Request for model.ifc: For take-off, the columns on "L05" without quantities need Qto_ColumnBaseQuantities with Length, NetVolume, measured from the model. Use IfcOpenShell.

First a look at what the model holds.

```python
import ifcopenshell
import ifcopenshell.util.element
import ifcopenshell.util.unit

model = ifcopenshell.open("model.ifc")
print(model.schema)
for unit_type in ("LENGTHUNIT", "AREAUNIT", "VOLUMEUNIT"):
    print(unit_type, ifcopenshell.util.unit.calculate_unit_scale(model, unit_type))
storey = next(s for s in model.by_type("IfcBuildingStorey") if s.Name == "L05")
columns = [e for e in ifcopenshell.util.element.get_decomposition(storey) if e.is_a("IfcColumn")]
for e in sorted(columns, key=lambda e: e.id()):
    print(e.id(), e.is_a(), e.Name, list(ifcopenshell.util.element.get_psets(e, qtos_only=True)), sep=" | ")
```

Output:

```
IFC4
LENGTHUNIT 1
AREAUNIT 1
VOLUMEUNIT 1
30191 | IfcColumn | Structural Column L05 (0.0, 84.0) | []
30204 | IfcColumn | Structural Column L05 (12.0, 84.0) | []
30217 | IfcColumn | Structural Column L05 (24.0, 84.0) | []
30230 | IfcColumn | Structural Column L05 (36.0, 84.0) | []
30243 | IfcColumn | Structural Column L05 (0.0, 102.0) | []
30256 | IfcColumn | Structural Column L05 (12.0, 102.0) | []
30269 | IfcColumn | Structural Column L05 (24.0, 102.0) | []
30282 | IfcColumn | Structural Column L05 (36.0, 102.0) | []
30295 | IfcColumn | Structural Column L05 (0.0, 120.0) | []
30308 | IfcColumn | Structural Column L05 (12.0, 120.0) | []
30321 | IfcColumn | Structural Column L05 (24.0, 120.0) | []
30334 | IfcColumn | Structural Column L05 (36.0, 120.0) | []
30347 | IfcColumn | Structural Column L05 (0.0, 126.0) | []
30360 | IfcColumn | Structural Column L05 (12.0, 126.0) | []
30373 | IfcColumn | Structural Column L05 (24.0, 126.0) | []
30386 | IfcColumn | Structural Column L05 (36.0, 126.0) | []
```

```python
import ifcopenshell
import ifcopenshell.api.pset
import ifcopenshell.geom
import ifcopenshell.util.element
import ifcopenshell.util.shape
import ifcopenshell.util.unit

model = ifcopenshell.open("model.ifc")
unit_scale = ifcopenshell.util.unit.calculate_unit_scale(model)
volume_scale = ifcopenshell.util.unit.calculate_unit_scale(model, "VOLUMEUNIT")
settings = ifcopenshell.geom.settings()

storey = next(s for s in model.by_type("IfcBuildingStorey") if s.Name == "L05")
columns = [e for e in ifcopenshell.util.element.get_decomposition(storey) if e.is_a("IfcColumn")]

for e in sorted(columns, key=lambda e: e.id()):
    if ifcopenshell.util.element.get_psets(e, qtos_only=True, should_inherit=False):
        continue
    # Geometry comes back in metres, in the element's own axes.
    shape = ifcopenshell.geom.create_shape(settings, e)
    values = {
        "Length": ifcopenshell.util.shape.get_z(shape.geometry) / unit_scale,
        "NetVolume": ifcopenshell.util.shape.get_volume(shape.geometry) / volume_scale,
    }
    qto = ifcopenshell.api.pset.add_qto(model, product=e, name="Qto_ColumnBaseQuantities")
    ifcopenshell.api.pset.edit_qto(model, qto=qto, properties=values)
    print(e.id(), {k: round(v, 3) for k, v in values.items()})

model.write("model_edited.ifc")
```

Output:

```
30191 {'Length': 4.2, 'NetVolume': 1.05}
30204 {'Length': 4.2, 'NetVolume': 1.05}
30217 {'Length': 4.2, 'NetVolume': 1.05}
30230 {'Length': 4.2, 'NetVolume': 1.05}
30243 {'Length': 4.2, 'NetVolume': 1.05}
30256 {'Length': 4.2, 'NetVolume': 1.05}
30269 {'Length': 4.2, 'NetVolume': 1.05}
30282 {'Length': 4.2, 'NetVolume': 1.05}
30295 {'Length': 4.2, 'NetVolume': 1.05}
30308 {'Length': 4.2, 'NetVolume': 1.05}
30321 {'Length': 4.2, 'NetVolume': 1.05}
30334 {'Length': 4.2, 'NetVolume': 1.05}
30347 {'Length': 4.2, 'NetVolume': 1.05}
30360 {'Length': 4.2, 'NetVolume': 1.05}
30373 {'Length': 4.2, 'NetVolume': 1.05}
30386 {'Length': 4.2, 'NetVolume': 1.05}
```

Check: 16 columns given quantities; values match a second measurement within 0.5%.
